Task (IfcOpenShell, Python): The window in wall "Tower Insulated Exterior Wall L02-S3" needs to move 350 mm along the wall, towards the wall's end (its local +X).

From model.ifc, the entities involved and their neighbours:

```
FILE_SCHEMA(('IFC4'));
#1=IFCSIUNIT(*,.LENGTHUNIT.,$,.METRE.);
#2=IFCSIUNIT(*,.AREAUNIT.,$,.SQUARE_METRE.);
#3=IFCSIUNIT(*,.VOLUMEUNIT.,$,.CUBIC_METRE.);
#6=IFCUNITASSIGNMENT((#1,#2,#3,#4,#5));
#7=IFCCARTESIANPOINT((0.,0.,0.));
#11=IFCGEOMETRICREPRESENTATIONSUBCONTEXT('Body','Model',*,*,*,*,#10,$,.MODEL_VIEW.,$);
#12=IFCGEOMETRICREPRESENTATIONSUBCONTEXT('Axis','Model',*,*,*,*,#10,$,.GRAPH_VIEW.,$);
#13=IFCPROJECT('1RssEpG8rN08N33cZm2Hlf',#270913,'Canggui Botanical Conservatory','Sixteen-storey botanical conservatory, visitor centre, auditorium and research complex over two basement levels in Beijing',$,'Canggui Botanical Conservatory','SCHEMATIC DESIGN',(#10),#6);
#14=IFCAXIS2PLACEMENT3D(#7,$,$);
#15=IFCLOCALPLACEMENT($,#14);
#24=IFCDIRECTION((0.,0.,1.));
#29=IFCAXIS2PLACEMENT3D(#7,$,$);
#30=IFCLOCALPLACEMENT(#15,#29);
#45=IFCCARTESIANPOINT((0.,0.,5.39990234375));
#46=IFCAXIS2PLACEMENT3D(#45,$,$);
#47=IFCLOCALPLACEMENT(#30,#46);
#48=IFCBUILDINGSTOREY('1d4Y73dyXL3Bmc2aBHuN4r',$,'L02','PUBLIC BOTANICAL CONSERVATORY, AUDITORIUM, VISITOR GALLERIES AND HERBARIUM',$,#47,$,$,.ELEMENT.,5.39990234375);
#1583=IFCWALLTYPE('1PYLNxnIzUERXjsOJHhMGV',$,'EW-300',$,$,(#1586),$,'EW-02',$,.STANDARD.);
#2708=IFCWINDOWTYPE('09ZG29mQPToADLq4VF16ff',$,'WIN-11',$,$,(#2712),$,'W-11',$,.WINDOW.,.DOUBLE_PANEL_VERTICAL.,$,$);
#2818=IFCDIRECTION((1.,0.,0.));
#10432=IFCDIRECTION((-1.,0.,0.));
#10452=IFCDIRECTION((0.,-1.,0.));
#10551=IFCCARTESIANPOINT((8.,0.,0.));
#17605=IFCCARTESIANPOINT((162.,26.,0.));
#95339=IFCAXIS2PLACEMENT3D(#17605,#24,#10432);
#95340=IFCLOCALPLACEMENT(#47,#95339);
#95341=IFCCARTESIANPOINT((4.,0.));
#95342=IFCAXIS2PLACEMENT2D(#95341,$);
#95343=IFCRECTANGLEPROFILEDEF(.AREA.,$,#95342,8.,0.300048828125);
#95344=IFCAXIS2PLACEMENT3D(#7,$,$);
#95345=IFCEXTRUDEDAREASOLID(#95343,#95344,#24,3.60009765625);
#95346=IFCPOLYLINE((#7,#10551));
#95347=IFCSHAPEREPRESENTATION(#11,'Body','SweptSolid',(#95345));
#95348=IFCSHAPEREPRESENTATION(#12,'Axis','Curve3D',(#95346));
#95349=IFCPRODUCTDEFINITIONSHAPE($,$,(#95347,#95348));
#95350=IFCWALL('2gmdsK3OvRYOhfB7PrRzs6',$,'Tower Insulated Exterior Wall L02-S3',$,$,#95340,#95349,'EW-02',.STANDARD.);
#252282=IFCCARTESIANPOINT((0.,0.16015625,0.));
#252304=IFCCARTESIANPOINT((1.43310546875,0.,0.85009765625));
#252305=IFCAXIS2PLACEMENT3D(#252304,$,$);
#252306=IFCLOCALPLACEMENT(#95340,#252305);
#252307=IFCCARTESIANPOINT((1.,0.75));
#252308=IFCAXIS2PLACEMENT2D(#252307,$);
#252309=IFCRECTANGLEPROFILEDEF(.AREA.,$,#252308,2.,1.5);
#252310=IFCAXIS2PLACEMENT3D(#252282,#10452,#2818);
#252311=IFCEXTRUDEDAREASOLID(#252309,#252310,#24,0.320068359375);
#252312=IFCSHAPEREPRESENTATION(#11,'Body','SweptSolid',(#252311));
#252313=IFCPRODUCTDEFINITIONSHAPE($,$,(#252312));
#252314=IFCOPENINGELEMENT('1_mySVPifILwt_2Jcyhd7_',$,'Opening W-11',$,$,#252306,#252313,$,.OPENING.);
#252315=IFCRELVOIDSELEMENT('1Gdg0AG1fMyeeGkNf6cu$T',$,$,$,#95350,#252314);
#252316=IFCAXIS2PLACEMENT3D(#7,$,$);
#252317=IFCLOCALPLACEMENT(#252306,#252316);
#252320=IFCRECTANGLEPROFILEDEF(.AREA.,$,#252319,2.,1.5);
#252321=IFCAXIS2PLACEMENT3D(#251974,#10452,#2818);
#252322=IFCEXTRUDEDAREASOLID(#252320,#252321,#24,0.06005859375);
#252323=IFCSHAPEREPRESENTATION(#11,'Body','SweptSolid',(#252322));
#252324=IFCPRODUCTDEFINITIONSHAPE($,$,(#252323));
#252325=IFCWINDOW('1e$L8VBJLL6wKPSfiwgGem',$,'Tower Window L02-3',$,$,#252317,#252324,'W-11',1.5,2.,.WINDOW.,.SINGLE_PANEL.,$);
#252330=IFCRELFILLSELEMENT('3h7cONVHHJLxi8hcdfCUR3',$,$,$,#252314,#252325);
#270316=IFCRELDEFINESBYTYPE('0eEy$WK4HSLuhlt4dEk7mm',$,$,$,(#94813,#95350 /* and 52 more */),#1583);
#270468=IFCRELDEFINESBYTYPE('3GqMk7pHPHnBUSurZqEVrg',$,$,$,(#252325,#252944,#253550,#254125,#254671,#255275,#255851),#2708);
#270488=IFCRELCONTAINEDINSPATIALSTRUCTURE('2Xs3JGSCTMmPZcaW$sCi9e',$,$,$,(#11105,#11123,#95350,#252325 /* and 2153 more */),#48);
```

```python
import ifcopenshell
import ifcopenshell.api.geometry
import ifcopenshell.util.placement
import ifcopenshell.util.unit

model = ifcopenshell.open("model.ifc")
unit_scale = ifcopenshell.util.unit.calculate_unit_scale(model)

window = model.by_guid("1e$L8VBJLL6wKPSfiwgGem")
opening = window.FillsVoids[0].RelatingOpeningElement
wall = opening.VoidsElements[0].RelatingBuildingElement

wall_matrix = ifcopenshell.util.placement.get_local_placement(wall.ObjectPlacement)
shift = wall_matrix[:3, 0] * 0.35 / unit_scale
before = ifcopenshell.util.placement.get_local_placement(window.ObjectPlacement)[:3, 3].copy()

# The window is placed relative to its opening, so it follows when the opening moves.
matrix = ifcopenshell.util.placement.get_local_placement(opening.ObjectPlacement)
matrix[:3, 3] += shift
ifcopenshell.api.geometry.edit_object_placement(
    model, product=opening, matrix=matrix, is_si=False, should_transform_children=True
)

after = ifcopenshell.util.placement.get_local_placement(window.ObjectPlacement)[:3, 3]
print("window moved by", (after - before).round(3) + 0.0)

model.write("model_updated.ifc")
```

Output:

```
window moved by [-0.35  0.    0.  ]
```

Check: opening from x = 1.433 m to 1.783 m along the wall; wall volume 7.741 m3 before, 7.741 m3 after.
